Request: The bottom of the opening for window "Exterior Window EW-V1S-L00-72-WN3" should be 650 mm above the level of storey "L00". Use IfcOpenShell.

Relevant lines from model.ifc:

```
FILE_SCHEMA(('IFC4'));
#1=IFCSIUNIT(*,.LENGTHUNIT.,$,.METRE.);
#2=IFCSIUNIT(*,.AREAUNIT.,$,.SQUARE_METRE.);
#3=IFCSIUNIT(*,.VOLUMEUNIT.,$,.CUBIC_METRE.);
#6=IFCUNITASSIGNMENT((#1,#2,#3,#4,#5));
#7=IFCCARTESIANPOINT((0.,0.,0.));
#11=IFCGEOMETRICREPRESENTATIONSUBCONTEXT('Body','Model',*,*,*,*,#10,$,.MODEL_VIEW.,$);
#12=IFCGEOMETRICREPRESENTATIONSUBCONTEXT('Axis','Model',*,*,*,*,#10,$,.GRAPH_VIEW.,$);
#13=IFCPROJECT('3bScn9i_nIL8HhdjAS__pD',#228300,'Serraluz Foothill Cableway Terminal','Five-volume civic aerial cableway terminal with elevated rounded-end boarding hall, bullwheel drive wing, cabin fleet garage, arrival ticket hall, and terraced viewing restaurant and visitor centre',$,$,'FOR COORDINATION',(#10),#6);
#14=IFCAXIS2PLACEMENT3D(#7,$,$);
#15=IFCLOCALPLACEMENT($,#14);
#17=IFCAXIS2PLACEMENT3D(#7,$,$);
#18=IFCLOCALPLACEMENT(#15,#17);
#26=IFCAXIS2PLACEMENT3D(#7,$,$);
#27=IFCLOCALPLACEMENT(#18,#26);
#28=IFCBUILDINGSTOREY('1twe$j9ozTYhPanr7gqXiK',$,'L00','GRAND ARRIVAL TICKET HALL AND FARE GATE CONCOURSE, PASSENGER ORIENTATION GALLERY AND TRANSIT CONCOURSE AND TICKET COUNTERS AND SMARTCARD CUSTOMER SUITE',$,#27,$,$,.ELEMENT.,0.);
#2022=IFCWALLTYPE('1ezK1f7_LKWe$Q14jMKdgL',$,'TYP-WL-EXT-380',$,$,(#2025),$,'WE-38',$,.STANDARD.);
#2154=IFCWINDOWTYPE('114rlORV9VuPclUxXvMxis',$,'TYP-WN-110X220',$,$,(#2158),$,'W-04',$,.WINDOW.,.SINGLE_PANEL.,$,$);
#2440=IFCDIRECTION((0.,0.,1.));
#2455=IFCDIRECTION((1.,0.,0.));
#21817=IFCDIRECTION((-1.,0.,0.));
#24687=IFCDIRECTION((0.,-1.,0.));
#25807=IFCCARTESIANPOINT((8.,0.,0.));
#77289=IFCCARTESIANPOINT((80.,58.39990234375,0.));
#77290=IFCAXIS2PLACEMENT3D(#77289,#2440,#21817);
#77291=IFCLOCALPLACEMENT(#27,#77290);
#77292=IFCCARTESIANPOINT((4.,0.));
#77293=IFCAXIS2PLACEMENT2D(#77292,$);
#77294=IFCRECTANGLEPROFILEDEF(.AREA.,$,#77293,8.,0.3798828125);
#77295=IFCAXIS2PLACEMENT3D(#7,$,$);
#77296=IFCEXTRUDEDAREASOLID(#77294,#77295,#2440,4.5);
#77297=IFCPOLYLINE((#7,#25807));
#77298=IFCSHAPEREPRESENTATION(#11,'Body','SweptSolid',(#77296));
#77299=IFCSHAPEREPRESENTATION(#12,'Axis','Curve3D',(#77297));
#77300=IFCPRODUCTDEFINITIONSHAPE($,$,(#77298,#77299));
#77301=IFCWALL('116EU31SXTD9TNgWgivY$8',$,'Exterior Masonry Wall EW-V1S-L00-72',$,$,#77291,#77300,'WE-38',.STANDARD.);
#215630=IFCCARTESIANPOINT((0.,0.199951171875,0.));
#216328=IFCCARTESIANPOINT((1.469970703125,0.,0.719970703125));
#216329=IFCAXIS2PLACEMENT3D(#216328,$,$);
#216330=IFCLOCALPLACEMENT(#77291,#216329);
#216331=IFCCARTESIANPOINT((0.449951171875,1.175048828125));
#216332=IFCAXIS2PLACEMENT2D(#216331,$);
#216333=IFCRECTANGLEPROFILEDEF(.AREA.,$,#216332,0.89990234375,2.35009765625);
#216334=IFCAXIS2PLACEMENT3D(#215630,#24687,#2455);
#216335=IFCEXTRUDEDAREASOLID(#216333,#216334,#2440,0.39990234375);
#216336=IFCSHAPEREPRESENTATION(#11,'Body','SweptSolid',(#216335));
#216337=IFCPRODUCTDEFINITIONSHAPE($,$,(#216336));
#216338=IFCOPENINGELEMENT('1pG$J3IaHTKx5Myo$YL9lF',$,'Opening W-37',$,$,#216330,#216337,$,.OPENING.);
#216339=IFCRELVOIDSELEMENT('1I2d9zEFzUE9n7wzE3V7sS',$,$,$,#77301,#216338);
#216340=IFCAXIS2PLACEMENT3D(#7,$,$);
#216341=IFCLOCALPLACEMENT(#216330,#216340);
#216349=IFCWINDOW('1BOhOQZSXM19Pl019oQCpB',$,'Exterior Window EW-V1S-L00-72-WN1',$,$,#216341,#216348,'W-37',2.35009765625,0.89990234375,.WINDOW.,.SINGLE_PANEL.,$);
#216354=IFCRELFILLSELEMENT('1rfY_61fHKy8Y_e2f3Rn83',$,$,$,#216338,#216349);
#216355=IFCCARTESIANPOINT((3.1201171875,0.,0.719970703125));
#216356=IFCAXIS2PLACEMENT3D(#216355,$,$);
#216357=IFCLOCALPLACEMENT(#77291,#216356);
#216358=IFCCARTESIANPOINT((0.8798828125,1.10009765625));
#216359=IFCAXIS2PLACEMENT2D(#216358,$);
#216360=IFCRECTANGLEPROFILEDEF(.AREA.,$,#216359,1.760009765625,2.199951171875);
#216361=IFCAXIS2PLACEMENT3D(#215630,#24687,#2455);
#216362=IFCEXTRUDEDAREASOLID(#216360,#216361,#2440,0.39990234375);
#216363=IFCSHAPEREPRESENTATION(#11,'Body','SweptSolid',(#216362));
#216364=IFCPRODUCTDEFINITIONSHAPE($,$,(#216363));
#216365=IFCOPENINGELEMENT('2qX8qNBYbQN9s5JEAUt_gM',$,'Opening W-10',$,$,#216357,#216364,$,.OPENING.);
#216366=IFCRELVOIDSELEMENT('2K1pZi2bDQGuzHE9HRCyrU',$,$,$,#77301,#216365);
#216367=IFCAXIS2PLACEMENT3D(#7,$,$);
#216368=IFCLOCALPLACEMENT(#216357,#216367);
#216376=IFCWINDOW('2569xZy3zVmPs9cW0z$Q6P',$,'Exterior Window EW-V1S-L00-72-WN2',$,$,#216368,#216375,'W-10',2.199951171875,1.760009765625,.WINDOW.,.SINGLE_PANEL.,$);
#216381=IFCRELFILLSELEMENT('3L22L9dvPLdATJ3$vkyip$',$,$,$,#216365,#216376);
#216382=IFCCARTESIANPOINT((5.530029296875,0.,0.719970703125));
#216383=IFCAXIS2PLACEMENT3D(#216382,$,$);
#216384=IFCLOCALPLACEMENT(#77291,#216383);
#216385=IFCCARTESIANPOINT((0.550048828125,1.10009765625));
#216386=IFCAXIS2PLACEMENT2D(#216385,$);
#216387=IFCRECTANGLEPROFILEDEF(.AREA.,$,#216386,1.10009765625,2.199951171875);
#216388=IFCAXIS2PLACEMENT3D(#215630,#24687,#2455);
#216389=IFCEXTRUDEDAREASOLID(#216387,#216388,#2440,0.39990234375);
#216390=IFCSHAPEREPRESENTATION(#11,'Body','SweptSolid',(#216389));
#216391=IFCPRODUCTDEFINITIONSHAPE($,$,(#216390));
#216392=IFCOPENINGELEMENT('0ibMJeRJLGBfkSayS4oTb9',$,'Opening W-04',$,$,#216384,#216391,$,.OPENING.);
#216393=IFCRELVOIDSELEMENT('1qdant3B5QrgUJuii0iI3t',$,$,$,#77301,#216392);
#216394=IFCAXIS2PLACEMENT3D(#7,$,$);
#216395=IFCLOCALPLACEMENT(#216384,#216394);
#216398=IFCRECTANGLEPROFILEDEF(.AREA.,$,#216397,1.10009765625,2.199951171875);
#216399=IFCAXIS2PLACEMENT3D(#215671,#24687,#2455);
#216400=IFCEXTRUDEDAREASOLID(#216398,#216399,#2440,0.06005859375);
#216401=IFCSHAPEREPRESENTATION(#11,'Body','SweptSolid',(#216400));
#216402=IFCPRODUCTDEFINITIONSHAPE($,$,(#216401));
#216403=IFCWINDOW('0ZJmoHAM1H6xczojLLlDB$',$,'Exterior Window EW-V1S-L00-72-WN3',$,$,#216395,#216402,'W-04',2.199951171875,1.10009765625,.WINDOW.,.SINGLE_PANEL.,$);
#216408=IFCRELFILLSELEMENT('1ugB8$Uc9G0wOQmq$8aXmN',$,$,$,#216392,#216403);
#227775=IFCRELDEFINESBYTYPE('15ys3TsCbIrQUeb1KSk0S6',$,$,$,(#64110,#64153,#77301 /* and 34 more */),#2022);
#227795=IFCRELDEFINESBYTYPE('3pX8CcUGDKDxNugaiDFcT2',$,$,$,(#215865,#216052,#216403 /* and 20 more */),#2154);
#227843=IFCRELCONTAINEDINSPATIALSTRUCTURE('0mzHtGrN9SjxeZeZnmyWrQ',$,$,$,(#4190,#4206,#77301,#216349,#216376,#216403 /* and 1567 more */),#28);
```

```python
import numpy as np
import ifcopenshell
import ifcopenshell.api.geometry
import ifcopenshell.geom
import ifcopenshell.util.element
import ifcopenshell.util.placement
import ifcopenshell.util.shape
import ifcopenshell.util.unit

model = ifcopenshell.open("model.ifc")
unit_scale = ifcopenshell.util.unit.calculate_unit_scale(model)

window = model.by_guid("0ZJmoHAM1H6xczojLLlDB$")
opening = window.FillsVoids[0].RelatingOpeningElement
storey = ifcopenshell.util.element.get_container(window, ifc_class="IfcBuildingStorey")
level = ifcopenshell.util.placement.get_local_placement(storey.ObjectPlacement)[2, 3]

# The opening's origin need not be at the sill, so measure its lowest point.
shape = ifcopenshell.geom.create_shape(ifcopenshell.geom.settings(), opening)
bottom = ifcopenshell.util.shape.get_shape_bottom_elevation(shape, shape.geometry) / unit_scale
dz = level + 0.65 / unit_scale - bottom

shift = np.array([0.0, 0.0, dz])
# The window is placed relative to its opening, so it follows when the opening moves.
matrix = ifcopenshell.util.placement.get_local_placement(opening.ObjectPlacement)
matrix[:3, 3] += shift
ifcopenshell.api.geometry.edit_object_placement(
    model, product=opening, matrix=matrix, is_si=False, should_transform_children=True
)

print(f"moved by {dz * unit_scale:+.3f} m")

model.write("model-out.ifc")
```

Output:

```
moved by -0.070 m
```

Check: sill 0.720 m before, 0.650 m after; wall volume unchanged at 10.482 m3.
